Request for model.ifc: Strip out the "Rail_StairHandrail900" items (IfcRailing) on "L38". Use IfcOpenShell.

First a look at what the model holds.

```python
import ifcopenshell
import ifcopenshell.util.element

model = ifcopenshell.open("model.ifc")
print(model.schema)
storey = next(s for s in model.by_type("IfcBuildingStorey") if s.Name == "L38")
railings = [e for e in ifcopenshell.util.element.get_decomposition(storey) if e.is_a("IfcRailing")]
seen = {}
for e in railings:
    element_type = ifcopenshell.util.element.get_type(e)
    name = element_type.Name if element_type not in (None, e) else None
    seen[name] = seen.get(name, 0) + 1
for name, count in sorted(seen.items(), key=str):
    print(count, "x", name)
```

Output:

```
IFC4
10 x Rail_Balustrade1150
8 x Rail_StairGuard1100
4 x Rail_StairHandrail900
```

```python
import ifcopenshell
import ifcopenshell.api.root
import ifcopenshell.util.element

model = ifcopenshell.open("model.ifc")

storey = next(s for s in model.by_type("IfcBuildingStorey") if s.Name == "L38")
railings = [e for e in ifcopenshell.util.element.get_decomposition(storey) if e.is_a("IfcRailing")]
targets = [e for e in railings if (t := ifcopenshell.util.element.get_type(e)) not in (None, e) and t.Name == "Rail_StairHandrail900"]

for e in targets:
    ifcopenshell.api.root.remove_product(model, product=e)
print(len(targets), "removed")

model.write("model_rev.ifc")
```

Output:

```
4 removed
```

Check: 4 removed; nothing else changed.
